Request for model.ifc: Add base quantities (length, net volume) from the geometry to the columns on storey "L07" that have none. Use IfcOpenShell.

First a look at what the model holds.

```python
import ifcopenshell
import ifcopenshell.util.element
import ifcopenshell.util.unit

model = ifcopenshell.open("model.ifc")
print(model.schema)
for unit_type in ("LENGTHUNIT", "AREAUNIT", "VOLUMEUNIT"):
    print(unit_type, ifcopenshell.util.unit.calculate_unit_scale(model, unit_type))
storey = next(s for s in model.by_type("IfcBuildingStorey") if s.Name == "L07")
columns = [e for e in ifcopenshell.util.element.get_decomposition(storey) if e.is_a("IfcColumn")]
for e in sorted(columns, key=lambda e: e.id()):
    print(e.id(), e.is_a(), e.Name, list(ifcopenshell.util.element.get_psets(e, qtos_only=True)), sep=" | ")
```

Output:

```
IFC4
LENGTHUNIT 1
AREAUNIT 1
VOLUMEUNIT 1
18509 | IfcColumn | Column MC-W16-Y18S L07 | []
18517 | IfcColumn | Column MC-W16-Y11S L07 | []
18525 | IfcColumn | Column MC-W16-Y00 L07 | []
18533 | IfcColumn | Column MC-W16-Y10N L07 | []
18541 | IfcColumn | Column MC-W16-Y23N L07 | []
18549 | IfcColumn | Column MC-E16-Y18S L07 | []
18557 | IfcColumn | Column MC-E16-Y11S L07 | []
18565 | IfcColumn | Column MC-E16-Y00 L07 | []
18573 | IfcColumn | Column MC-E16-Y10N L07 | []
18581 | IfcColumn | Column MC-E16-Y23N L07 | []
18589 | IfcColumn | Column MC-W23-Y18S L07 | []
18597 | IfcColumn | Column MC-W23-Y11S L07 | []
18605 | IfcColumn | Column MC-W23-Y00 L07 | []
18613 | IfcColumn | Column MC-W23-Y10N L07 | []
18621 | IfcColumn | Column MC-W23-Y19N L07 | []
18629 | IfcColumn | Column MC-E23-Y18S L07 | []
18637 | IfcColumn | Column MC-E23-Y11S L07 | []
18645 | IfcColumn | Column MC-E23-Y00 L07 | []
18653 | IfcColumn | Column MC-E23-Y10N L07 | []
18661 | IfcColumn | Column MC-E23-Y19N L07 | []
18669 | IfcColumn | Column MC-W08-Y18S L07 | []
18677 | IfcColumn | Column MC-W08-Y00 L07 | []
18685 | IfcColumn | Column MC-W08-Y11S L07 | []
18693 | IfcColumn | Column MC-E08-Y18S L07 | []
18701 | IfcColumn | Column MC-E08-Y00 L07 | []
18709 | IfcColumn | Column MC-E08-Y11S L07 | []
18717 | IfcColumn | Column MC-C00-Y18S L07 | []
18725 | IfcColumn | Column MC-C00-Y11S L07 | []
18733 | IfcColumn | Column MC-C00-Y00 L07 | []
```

```python
import ifcopenshell
import ifcopenshell.api.pset
import ifcopenshell.geom
import ifcopenshell.util.element
import ifcopenshell.util.shape
import ifcopenshell.util.unit

model = ifcopenshell.open("model.ifc")
unit_scale = ifcopenshell.util.unit.calculate_unit_scale(model)
volume_scale = ifcopenshell.util.unit.calculate_unit_scale(model, "VOLUMEUNIT")
settings = ifcopenshell.geom.settings()

storey = next(s for s in model.by_type("IfcBuildingStorey") if s.Name == "L07")
columns = [e for e in ifcopenshell.util.element.get_decomposition(storey) if e.is_a("IfcColumn")]

for e in sorted(columns, key=lambda e: e.id()):
    if ifcopenshell.util.element.get_psets(e, qtos_only=True, should_inherit=False):
        continue
    # Geometry comes back in metres, in the element's own axes.
    shape = ifcopenshell.geom.create_shape(settings, e)
    values = {
        "Length": ifcopenshell.util.shape.get_z(shape.geometry) / unit_scale,
        "NetVolume": ifcopenshell.util.shape.get_volume(shape.geometry) / volume_scale,
    }
    qto = ifcopenshell.api.pset.add_qto(model, product=e, name="Qto_ColumnBaseQuantities")
    ifcopenshell.api.pset.edit_qto(model, qto=qto, properties=values)
    print(e.id(), {k: round(v, 3) for k, v in values.items()})

model.write("model-out.ifc")
```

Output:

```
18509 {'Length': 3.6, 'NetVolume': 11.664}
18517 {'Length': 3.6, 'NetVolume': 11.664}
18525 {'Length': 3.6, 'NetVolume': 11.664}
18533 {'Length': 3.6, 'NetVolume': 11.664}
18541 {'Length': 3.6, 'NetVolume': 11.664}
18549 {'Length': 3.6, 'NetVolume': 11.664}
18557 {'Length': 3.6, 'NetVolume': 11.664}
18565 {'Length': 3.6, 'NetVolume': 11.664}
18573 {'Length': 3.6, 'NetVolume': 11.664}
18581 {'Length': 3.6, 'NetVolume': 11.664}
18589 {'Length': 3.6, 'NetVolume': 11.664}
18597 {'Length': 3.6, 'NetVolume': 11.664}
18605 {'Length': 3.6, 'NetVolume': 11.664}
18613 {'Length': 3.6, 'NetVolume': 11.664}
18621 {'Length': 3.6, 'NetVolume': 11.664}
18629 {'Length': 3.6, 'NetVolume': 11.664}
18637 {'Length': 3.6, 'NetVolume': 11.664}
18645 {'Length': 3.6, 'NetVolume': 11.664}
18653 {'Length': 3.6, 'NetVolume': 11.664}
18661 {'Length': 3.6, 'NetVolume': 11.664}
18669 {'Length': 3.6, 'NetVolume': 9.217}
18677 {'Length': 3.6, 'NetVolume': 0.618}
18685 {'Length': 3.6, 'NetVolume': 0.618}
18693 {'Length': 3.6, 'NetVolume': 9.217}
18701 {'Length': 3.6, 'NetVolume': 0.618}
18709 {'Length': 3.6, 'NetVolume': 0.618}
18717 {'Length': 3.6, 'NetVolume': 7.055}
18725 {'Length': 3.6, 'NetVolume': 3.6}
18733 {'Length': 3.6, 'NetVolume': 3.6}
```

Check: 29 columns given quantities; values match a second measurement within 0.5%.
